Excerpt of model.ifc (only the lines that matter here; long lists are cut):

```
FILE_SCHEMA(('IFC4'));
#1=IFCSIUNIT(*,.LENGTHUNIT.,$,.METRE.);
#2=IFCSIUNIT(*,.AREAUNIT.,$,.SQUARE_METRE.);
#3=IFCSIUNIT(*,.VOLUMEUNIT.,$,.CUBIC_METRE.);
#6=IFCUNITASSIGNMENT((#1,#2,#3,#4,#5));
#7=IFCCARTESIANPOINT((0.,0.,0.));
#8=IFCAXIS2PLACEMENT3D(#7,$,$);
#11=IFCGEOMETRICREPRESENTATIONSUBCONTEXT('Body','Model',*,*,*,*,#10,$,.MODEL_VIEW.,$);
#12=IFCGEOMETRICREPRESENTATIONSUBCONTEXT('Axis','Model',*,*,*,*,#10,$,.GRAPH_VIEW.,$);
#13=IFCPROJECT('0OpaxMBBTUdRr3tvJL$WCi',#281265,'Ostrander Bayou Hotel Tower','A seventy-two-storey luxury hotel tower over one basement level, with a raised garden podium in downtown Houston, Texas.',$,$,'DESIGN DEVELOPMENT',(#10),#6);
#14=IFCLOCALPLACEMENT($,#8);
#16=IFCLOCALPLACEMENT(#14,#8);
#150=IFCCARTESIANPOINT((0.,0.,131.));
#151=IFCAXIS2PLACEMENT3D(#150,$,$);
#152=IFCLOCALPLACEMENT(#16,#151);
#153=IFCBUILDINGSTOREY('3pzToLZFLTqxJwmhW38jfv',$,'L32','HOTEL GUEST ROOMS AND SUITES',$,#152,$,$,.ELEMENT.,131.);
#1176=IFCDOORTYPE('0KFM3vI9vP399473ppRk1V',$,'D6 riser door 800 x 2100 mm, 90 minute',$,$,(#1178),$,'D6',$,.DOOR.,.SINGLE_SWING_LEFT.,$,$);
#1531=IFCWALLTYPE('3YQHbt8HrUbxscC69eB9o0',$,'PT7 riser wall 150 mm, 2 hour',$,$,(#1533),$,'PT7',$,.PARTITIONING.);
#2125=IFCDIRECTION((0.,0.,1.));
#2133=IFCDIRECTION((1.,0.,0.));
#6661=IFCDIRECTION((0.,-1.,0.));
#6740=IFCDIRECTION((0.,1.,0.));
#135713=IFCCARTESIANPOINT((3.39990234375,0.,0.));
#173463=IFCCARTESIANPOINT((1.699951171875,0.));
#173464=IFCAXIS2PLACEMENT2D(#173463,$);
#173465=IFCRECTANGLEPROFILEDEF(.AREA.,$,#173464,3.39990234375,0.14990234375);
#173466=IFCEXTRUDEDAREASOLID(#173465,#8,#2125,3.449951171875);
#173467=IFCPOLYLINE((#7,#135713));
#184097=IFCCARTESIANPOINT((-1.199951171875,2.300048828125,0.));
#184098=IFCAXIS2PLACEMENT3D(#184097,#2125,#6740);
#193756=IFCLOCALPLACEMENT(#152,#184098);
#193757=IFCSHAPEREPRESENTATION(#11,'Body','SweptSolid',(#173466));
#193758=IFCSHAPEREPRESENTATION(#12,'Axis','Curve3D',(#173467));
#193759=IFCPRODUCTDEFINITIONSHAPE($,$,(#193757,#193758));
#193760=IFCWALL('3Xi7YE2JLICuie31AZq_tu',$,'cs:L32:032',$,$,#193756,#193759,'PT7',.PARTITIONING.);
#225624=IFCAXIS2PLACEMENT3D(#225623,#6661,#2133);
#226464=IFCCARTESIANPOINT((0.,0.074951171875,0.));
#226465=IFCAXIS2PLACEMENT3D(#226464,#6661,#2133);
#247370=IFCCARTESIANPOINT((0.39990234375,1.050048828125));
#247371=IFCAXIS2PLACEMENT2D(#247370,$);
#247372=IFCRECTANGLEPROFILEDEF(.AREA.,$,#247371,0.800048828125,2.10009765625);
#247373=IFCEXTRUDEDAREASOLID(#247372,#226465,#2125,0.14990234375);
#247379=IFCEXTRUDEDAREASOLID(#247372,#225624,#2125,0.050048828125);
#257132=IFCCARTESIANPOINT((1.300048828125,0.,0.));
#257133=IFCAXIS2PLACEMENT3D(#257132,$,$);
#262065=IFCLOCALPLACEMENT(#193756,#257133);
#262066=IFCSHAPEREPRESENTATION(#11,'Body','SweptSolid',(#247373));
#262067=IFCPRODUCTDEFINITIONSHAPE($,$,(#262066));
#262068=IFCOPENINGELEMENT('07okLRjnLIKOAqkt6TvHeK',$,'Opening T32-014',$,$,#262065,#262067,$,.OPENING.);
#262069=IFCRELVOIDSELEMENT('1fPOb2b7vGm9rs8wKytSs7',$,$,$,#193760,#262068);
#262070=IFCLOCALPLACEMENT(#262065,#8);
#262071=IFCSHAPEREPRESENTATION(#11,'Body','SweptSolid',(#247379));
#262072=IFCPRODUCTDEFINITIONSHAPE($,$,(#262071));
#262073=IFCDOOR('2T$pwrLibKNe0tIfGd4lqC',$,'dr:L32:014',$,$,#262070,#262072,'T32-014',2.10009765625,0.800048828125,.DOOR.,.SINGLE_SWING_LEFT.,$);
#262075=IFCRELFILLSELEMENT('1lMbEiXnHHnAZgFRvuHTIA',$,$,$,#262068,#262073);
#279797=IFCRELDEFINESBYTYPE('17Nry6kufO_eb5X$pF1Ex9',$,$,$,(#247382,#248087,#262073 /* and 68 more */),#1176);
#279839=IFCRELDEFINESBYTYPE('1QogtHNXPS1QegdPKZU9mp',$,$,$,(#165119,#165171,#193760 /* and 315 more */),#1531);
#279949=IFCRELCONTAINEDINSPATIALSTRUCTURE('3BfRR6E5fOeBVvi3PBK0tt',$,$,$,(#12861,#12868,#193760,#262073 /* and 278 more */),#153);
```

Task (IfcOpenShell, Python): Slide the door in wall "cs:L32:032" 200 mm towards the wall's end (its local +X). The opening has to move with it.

```python
import ifcopenshell
import ifcopenshell.api.geometry
import ifcopenshell.util.placement
import ifcopenshell.util.unit

model = ifcopenshell.open("model.ifc")
unit_scale = ifcopenshell.util.unit.calculate_unit_scale(model)

door = model.by_guid("2T$pwrLibKNe0tIfGd4lqC")
opening = door.FillsVoids[0].RelatingOpeningElement
wall = opening.VoidsElements[0].RelatingBuildingElement

wall_matrix = ifcopenshell.util.placement.get_local_placement(wall.ObjectPlacement)
shift = wall_matrix[:3, 0] * 0.2 / unit_scale
before = ifcopenshell.util.placement.get_local_placement(door.ObjectPlacement)[:3, 3].copy()

# The door is placed relative to its opening, so it follows when the opening moves.
matrix = ifcopenshell.util.placement.get_local_placement(opening.ObjectPlacement)
matrix[:3, 3] += shift
ifcopenshell.api.geometry.edit_object_placement(
    model, product=opening, matrix=matrix, is_si=False, should_transform_children=True
)

after = ifcopenshell.util.placement.get_local_placement(door.ObjectPlacement)[:3, 3]
print("door moved by", (after - before).round(3) + 0.0)

model.write("model_updated.ifc")
```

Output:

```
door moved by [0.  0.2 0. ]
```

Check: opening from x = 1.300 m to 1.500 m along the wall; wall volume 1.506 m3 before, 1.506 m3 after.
